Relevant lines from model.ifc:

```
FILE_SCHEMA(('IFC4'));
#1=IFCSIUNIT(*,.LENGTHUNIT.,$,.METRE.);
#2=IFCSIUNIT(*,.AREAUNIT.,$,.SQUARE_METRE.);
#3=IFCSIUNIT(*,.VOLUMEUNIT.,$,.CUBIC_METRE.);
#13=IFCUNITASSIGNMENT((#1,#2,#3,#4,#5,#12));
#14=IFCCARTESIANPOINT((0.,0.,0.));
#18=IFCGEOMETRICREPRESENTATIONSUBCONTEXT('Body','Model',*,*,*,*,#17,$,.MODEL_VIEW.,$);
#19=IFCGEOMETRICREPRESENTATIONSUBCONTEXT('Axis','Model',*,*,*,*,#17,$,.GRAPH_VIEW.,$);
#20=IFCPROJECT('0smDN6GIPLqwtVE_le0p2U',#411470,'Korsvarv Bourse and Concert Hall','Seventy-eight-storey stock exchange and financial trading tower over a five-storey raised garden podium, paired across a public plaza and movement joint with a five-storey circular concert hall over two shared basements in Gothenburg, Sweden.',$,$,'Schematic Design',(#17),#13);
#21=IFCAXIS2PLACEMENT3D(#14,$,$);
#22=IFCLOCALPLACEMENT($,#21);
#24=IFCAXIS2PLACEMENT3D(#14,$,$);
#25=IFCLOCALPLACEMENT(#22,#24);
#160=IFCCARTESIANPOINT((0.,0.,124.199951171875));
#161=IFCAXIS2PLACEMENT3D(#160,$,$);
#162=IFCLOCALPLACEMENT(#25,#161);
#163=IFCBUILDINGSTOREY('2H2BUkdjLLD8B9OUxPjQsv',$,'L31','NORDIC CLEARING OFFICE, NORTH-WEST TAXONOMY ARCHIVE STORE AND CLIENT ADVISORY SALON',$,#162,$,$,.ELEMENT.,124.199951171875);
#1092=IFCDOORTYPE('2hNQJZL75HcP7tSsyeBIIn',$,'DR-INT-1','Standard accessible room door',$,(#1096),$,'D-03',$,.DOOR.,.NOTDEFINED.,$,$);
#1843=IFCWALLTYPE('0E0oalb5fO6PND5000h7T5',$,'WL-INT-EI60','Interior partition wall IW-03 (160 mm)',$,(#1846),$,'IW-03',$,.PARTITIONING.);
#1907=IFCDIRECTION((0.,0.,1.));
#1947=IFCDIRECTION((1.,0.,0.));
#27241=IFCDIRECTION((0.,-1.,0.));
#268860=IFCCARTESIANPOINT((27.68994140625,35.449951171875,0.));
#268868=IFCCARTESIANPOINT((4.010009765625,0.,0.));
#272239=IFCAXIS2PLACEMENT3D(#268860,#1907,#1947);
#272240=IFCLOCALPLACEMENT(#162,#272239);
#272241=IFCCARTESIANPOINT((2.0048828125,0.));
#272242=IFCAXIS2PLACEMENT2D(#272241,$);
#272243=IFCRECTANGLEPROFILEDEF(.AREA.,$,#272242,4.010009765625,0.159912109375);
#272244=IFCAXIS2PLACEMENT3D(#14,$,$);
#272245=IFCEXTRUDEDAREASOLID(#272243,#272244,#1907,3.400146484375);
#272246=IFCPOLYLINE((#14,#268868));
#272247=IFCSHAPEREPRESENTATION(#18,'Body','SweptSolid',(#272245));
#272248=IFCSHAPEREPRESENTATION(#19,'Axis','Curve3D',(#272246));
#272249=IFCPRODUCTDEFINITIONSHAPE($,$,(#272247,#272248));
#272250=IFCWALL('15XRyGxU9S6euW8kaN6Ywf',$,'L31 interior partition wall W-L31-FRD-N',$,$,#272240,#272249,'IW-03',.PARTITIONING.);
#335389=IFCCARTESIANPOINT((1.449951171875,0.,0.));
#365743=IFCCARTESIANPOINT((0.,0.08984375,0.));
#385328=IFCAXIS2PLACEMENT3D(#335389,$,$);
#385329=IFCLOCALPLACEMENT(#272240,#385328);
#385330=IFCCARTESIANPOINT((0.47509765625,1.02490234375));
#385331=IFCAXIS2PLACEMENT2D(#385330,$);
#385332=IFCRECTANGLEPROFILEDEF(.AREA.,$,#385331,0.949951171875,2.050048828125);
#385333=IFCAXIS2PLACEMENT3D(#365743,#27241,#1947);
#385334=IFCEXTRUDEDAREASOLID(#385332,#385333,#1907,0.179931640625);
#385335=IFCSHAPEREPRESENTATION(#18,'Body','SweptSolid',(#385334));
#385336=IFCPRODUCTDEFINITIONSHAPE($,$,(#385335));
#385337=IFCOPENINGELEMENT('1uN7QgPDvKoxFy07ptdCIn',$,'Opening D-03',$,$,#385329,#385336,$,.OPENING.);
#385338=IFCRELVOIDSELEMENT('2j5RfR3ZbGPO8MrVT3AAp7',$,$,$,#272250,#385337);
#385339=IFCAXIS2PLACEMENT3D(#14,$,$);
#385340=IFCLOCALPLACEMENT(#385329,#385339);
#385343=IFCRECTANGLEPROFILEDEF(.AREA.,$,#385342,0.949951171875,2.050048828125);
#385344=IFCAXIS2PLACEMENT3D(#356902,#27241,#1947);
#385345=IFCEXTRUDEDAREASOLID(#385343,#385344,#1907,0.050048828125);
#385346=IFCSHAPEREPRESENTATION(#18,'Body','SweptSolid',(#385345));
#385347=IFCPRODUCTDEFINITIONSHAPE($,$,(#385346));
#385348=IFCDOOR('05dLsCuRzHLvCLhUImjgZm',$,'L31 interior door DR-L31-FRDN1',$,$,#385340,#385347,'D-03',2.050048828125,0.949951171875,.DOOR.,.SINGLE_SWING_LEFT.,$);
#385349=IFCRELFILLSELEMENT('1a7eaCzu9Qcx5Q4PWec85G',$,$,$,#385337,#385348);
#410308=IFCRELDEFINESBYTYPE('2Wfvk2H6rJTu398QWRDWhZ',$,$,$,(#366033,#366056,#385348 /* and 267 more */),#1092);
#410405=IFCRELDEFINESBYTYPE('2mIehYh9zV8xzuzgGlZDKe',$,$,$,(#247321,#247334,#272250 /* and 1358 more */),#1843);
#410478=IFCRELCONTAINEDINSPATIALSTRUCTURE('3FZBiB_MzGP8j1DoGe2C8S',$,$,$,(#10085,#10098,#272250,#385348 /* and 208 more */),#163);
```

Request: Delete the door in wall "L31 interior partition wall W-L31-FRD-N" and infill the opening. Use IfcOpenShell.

```python
import ifcopenshell
import ifcopenshell.api.feature
import ifcopenshell.api.root
import ifcopenshell.geom
import ifcopenshell.util.shape

model = ifcopenshell.open("model.ifc")
settings = ifcopenshell.geom.settings()


def volume(element):
    """Net volume in cubic metres, openings subtracted."""
    shape = ifcopenshell.geom.create_shape(settings, element)
    return ifcopenshell.util.shape.get_volume(shape.geometry)


door = model.by_guid("05dLsCuRzHLvCLhUImjgZm")
opening = door.FillsVoids[0].RelatingOpeningElement
wall = opening.VoidsElements[0].RelatingBuildingElement
before = volume(wall)

ifcopenshell.api.root.remove_product(model, product=door)
ifcopenshell.api.feature.remove_feature(model, feature=opening)

after = volume(wall)

print(f"wall volume {before:.3f} -> {after:.3f} m3")

model.write("model_edited.ifc")
```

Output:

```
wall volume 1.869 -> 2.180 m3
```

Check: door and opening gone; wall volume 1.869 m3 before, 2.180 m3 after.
